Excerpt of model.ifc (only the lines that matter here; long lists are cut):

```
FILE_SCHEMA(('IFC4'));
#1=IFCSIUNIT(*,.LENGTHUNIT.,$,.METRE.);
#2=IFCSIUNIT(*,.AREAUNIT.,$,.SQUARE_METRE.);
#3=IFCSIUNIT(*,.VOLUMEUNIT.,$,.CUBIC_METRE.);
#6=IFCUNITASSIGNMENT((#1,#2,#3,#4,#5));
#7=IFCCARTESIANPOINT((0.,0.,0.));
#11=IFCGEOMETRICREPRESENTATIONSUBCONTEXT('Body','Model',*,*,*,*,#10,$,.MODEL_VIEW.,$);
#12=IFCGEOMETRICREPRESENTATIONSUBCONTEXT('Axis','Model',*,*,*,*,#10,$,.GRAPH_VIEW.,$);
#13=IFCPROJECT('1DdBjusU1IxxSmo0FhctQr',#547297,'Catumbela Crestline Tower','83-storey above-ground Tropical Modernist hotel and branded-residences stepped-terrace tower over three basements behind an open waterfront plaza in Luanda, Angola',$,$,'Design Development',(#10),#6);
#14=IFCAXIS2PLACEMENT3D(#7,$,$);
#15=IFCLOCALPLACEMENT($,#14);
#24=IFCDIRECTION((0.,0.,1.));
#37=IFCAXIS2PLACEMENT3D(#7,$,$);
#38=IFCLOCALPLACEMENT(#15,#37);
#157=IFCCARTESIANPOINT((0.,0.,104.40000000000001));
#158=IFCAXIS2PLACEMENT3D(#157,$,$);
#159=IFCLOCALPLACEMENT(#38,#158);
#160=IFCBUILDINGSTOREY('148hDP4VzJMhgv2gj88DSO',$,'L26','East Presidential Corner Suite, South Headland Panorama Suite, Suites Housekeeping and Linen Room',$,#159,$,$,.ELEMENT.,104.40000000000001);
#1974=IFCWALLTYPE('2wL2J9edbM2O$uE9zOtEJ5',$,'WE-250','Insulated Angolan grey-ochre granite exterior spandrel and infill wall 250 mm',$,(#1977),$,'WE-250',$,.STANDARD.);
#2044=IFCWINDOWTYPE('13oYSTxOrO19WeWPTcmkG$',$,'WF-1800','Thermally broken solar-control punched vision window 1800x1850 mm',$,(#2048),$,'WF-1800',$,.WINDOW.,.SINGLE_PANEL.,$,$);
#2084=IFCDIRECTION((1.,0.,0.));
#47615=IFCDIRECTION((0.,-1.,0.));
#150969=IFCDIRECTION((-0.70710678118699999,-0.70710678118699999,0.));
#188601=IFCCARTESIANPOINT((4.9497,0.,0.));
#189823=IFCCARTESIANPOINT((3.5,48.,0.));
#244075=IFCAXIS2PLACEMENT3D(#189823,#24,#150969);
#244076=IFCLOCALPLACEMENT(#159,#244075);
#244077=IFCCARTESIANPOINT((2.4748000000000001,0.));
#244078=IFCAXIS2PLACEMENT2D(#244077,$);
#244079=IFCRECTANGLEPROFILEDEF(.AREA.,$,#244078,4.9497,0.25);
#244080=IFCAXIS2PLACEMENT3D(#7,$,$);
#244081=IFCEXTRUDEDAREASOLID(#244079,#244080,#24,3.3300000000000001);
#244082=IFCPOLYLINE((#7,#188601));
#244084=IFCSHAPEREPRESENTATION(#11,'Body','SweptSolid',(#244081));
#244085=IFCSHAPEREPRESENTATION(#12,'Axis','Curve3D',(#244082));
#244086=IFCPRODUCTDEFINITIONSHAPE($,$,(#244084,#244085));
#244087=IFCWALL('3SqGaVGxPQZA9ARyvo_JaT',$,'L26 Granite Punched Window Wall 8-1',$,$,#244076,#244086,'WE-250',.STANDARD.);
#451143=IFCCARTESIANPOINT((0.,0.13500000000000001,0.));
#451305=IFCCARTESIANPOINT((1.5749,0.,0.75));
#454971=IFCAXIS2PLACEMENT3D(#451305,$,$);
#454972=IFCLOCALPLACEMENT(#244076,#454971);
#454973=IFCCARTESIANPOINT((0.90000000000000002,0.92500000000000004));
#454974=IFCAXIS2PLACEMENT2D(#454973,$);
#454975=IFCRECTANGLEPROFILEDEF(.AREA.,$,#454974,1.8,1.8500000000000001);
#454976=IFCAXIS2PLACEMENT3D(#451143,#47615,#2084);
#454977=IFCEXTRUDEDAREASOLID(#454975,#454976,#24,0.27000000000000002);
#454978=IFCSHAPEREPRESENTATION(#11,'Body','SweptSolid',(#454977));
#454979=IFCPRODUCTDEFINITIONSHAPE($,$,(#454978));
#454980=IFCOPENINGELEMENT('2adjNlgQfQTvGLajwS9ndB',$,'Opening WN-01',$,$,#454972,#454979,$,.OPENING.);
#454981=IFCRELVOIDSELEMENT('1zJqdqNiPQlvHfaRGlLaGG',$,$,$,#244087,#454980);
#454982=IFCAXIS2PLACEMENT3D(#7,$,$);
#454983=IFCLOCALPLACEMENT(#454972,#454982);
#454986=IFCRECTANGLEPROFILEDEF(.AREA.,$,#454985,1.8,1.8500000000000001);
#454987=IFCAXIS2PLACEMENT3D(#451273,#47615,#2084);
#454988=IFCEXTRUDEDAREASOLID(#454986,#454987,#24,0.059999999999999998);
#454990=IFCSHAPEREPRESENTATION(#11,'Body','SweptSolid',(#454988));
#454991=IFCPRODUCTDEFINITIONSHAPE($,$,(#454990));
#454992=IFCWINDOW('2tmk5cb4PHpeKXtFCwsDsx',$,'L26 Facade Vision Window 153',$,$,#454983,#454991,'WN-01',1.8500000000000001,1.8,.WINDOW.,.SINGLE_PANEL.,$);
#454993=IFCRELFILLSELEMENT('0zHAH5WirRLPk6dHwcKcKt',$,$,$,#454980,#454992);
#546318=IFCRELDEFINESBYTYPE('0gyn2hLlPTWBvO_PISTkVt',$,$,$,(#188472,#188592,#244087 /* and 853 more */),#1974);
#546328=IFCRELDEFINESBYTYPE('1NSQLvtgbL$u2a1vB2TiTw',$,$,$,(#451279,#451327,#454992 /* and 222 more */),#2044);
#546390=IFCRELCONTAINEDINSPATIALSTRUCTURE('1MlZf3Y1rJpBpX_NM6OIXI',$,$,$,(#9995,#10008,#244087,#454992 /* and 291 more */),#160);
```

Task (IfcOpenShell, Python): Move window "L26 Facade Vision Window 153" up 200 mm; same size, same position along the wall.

```python
import numpy as np
import ifcopenshell
import ifcopenshell.api.geometry
import ifcopenshell.util.placement
import ifcopenshell.util.unit

model = ifcopenshell.open("model.ifc")
unit_scale = ifcopenshell.util.unit.calculate_unit_scale(model)

window = model.by_guid("2tmk5cb4PHpeKXtFCwsDsx")
opening = window.FillsVoids[0].RelatingOpeningElement
dz = 0.2 / unit_scale

shift = np.array([0.0, 0.0, dz])
# The window is placed relative to its opening, so it follows when the opening moves.
matrix = ifcopenshell.util.placement.get_local_placement(opening.ObjectPlacement)
matrix[:3, 3] += shift
ifcopenshell.api.geometry.edit_object_placement(
    model, product=opening, matrix=matrix, is_si=False, should_transform_children=True
)

print(f"moved by {dz * unit_scale:+.3f} m")

model.write("model_rev.ifc")
```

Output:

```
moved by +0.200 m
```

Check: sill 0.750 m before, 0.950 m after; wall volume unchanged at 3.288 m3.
